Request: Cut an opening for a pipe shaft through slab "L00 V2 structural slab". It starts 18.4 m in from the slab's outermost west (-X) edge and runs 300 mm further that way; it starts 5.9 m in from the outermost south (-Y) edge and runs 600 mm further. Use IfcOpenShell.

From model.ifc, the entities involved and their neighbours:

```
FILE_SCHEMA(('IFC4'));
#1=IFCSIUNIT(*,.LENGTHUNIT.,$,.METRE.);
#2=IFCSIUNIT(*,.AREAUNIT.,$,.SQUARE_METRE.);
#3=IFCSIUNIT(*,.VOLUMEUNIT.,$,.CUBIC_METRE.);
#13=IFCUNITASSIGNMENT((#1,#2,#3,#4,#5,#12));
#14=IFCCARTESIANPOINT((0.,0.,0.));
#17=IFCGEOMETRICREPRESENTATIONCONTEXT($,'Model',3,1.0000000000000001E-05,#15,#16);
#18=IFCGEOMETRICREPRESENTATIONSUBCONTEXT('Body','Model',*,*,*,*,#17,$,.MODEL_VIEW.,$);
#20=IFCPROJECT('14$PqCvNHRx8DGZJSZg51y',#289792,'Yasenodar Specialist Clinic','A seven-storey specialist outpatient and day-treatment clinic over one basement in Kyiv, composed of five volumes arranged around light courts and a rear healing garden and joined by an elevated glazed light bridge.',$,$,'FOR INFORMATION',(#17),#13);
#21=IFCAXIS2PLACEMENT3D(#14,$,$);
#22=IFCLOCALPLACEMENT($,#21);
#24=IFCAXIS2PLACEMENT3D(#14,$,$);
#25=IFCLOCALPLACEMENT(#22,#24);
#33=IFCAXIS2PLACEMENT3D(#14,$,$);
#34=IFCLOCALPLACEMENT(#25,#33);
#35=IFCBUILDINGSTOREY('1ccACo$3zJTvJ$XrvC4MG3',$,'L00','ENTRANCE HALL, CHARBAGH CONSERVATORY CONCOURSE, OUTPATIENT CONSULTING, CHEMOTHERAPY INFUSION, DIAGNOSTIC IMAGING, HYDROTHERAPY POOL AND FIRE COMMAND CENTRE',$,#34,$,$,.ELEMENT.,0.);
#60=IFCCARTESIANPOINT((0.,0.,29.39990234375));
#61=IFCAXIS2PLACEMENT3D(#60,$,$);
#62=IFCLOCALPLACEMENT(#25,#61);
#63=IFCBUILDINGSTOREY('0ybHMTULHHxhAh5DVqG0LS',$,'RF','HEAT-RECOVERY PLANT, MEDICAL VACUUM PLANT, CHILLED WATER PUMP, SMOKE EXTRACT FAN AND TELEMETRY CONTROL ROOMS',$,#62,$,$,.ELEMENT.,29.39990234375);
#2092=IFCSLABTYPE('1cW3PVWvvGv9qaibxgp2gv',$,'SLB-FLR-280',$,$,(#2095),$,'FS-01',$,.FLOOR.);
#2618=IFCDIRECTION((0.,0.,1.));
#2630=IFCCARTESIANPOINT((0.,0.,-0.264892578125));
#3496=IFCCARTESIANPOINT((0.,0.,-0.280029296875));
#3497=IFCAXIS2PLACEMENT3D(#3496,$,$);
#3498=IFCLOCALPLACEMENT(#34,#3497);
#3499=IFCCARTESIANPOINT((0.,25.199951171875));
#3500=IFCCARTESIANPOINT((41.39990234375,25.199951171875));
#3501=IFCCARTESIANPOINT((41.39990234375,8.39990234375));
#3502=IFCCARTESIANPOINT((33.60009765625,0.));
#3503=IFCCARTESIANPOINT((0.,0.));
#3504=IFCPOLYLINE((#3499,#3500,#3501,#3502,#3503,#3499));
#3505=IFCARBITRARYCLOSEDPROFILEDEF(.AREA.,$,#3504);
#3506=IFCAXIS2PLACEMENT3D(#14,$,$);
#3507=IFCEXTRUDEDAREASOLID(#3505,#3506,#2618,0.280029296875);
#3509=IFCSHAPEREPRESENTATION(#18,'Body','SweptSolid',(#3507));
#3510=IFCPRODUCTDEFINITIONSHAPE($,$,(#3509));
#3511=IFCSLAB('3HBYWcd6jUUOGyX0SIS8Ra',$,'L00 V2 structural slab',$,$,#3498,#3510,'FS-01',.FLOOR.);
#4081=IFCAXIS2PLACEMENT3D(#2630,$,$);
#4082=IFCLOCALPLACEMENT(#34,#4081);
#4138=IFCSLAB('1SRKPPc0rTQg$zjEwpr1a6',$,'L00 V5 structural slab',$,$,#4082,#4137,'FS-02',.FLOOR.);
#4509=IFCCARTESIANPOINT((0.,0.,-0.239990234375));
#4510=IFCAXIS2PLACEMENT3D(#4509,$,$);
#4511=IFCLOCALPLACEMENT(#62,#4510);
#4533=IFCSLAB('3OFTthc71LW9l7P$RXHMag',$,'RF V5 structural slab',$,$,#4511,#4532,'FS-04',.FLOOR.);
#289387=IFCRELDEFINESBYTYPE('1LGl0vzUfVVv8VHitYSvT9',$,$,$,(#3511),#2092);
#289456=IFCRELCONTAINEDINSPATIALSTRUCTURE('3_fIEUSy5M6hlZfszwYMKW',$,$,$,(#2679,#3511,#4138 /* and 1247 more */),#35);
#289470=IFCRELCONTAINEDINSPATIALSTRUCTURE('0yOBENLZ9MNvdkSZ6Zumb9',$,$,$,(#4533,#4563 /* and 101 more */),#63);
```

```python
import numpy as np
import ifcopenshell
import ifcopenshell.api.feature
import ifcopenshell.api.geometry
import ifcopenshell.api.root
import ifcopenshell.geom
import ifcopenshell.util.placement
import ifcopenshell.util.representation
import ifcopenshell.util.shape
import ifcopenshell.util.unit

model = ifcopenshell.open("model.ifc")
unit_scale = ifcopenshell.util.unit.calculate_unit_scale(model)
settings = ifcopenshell.geom.settings()


def volume(element):
    """Net volume in cubic metres, openings subtracted."""
    shape = ifcopenshell.geom.create_shape(settings, element)
    return ifcopenshell.util.shape.get_volume(shape.geometry)


slab = model.by_id(3511)
before = volume(slab)

# Extent in the slab's own axes, in metres. The edges named are its -X and -Y sides.
slab_shape = ifcopenshell.geom.create_shape(settings, slab)
vertices = ifcopenshell.util.shape.get_vertices(slab_shape.geometry)
x_min, y_min, bottom = vertices.min(axis=0)
top = vertices[:, 2].max()

opening = ifcopenshell.api.root.create_entity(model, ifc_class="IfcOpeningElement", name="Pipe shaft opening", predefined_type="OPENING")
context = ifcopenshell.util.representation.get_context(model, "Model", "Body", "MODEL_VIEW")
width, depth = 0.3, 0.6
outline = [(0.0, 0.0), (width, 0.0), (width, depth), (0.0, depth), (0.0, 0.0)]
# Overshoot both faces by 50 mm so the cut is clean.
shape = ifcopenshell.api.geometry.add_slab_representation(
    model, context=context, depth=top - bottom + 0.1, polyline=outline
)
ifcopenshell.api.geometry.assign_representation(model, product=opening, representation=shape)

matrix = ifcopenshell.util.placement.get_local_placement(slab.ObjectPlacement)
matrix[:, 3] = matrix @ np.append(np.array([x_min + 18.4, y_min + 5.9, bottom - 0.05]) / unit_scale, 1.0)
ifcopenshell.api.geometry.edit_object_placement(model, product=opening, matrix=matrix, is_si=False)
ifcopenshell.api.feature.add_feature(model, feature=opening, element=slab)

after = volume(slab)

print(f"slab volume {before:.3f} -> {after:.3f} m3")

model.write("model_updated.ifc")
```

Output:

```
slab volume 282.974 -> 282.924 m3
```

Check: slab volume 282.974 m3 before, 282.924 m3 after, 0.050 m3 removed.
